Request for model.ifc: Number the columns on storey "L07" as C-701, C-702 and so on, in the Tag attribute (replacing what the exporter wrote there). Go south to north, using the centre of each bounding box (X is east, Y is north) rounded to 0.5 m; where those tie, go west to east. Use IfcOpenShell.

First a look at what the model holds.

```python
import ifcopenshell
import ifcopenshell.util.element
import ifcopenshell.util.placement

model = ifcopenshell.open("model.ifc")
print(model.schema)
storey = next(s for s in model.by_type("IfcBuildingStorey") if s.Name == "L07")
columns = [e for e in ifcopenshell.util.element.get_decomposition(storey) if e.is_a("IfcColumn")]
for e in sorted(columns, key=lambda e: e.id()):
    origin = ifcopenshell.util.placement.get_local_placement(e.ObjectPlacement)[:3, 3]
    print(e.id(), e.Tag, e.Name, origin.round(2) + 0.0, sep=" | ")
```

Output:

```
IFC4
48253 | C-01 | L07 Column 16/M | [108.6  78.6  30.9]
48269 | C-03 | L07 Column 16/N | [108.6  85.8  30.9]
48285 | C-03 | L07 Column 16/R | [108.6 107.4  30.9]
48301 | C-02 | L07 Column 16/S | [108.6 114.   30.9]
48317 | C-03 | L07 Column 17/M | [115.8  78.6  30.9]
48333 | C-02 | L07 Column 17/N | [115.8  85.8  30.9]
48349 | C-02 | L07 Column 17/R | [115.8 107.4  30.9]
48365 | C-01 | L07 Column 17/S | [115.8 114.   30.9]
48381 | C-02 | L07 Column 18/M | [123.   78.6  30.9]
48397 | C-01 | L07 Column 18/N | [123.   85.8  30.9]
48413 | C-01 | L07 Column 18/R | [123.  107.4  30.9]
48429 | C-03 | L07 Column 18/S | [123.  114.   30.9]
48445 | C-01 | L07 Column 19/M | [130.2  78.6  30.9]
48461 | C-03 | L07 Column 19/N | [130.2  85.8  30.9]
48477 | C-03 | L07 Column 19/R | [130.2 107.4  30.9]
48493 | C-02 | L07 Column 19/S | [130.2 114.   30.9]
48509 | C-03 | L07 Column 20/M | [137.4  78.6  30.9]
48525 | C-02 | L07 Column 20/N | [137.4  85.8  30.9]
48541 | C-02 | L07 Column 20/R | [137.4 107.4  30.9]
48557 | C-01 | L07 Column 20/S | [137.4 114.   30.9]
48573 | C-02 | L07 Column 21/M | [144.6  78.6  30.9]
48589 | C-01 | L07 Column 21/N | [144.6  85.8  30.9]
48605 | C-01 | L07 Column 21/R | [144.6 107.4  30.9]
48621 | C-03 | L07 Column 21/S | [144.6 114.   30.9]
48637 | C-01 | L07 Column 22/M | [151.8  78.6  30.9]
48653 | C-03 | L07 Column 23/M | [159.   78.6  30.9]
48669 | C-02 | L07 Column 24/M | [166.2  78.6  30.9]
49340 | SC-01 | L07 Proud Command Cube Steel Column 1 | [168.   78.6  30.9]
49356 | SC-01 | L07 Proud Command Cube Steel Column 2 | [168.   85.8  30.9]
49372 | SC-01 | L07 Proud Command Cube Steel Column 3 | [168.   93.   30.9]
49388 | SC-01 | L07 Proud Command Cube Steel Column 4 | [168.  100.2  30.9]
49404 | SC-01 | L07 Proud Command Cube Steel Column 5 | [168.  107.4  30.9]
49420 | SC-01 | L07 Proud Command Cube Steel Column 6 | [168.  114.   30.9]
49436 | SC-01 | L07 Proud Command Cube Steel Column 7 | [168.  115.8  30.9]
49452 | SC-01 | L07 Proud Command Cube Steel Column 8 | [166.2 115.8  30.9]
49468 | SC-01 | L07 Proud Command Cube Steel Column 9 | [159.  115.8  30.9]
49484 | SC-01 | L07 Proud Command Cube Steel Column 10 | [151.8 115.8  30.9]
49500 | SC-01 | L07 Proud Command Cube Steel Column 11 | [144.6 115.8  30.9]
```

```python
import ifcopenshell
import ifcopenshell.geom
import ifcopenshell.util.element
import ifcopenshell.util.shape

model = ifcopenshell.open("model.ifc")
settings = ifcopenshell.geom.settings()
settings.set("use-world-coords", True)


def centre(element):
    shape = ifcopenshell.geom.create_shape(settings, element)
    return ifcopenshell.util.shape.get_bbox_centroid(shape.geometry)


storey = next(s for s in model.by_type("IfcBuildingStorey") if s.Name == "L07")
columns = [e for e in ifcopenshell.util.element.get_decomposition(storey) if e.is_a("IfcColumn")]

# Insertion points can sit at a corner or the storey origin, so sort by the geometry (in metres).
centres = {e: centre(e) for e in columns}
columns.sort(key=lambda e: (round(centres[e][1] / 0.5), centres[e][0]))

for i, e in enumerate(columns, start=1):
    number = f"C-7{i:02d}"
    e.Tag = number
    print(e.id(), number)

model.write("model_edited.ifc")
```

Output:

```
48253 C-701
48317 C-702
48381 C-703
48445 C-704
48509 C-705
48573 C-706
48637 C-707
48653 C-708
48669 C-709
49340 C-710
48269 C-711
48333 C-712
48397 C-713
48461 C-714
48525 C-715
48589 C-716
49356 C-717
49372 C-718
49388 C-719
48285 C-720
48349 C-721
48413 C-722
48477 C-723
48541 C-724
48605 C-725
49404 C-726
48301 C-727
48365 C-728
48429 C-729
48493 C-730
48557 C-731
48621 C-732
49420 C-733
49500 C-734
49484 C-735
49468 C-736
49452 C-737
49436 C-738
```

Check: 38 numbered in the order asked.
